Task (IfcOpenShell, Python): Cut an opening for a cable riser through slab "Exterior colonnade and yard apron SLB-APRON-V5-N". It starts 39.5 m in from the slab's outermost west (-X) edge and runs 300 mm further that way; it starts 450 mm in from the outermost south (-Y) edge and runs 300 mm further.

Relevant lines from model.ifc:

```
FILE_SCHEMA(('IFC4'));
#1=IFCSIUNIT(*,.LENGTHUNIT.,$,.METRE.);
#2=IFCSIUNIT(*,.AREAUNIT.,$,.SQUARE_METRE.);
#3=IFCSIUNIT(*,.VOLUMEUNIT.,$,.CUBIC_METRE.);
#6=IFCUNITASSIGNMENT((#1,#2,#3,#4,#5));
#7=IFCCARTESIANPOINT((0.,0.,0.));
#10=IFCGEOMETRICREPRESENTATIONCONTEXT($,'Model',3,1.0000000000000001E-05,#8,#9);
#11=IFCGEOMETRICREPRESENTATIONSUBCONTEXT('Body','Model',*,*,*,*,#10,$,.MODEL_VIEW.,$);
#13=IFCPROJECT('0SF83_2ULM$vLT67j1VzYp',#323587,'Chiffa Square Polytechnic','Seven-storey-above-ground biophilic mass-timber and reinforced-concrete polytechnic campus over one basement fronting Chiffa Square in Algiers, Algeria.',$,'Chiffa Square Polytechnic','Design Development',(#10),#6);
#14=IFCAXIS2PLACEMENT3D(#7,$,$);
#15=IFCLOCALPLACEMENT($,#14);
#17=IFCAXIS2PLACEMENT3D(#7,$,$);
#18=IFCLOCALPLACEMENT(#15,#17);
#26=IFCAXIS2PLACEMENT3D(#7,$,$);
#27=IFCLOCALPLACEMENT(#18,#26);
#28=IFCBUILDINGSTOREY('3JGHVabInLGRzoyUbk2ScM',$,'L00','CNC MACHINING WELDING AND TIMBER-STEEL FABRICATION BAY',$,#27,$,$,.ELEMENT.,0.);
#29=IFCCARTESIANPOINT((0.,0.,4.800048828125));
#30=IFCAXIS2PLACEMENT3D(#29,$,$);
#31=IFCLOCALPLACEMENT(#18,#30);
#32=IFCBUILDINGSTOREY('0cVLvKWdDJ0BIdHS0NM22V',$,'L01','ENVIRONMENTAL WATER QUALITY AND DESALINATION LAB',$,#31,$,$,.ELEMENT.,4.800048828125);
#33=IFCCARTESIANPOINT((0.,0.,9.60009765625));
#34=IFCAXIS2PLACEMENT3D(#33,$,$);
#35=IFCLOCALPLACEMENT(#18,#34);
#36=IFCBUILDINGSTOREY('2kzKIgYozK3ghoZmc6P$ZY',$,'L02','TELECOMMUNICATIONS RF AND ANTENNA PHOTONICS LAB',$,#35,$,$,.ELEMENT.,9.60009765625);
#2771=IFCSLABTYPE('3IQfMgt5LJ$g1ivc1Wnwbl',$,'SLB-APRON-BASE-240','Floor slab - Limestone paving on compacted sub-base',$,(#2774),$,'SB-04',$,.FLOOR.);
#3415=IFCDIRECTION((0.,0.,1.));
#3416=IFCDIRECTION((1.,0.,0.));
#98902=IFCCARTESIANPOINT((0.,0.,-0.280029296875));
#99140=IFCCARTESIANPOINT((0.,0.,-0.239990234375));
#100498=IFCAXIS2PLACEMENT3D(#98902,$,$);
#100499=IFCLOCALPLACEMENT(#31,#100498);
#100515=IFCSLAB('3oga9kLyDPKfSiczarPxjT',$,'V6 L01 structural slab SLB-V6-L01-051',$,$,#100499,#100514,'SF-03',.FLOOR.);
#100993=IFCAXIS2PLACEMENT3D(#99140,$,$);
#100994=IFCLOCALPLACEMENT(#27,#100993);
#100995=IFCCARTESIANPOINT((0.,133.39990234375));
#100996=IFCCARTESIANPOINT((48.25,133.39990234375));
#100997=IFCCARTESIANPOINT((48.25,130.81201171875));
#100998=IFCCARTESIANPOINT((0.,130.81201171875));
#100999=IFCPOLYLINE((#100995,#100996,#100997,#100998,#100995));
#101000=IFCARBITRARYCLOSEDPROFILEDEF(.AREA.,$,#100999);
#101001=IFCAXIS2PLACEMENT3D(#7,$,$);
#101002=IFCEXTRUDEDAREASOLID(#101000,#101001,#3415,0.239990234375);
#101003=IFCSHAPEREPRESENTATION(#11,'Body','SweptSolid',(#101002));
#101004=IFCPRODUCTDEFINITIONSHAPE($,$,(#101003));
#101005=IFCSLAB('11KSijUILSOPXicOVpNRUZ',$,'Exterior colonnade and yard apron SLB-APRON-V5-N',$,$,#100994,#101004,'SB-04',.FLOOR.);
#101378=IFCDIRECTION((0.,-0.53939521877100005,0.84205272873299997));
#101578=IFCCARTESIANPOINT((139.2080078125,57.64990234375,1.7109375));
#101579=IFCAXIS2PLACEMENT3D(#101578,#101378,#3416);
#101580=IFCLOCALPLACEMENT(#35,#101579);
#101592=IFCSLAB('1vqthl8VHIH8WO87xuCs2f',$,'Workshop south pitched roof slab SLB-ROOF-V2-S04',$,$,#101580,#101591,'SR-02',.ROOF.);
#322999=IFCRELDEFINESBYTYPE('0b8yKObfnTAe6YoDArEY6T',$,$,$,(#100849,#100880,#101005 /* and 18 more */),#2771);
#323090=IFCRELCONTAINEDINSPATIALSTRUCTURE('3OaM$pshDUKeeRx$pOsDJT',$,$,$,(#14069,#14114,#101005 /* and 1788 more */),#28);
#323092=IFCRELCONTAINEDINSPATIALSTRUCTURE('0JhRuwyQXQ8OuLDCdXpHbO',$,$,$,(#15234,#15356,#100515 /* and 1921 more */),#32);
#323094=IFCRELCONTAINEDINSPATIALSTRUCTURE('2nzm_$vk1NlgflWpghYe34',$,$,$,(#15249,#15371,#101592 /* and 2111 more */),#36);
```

```python
import numpy as np
import ifcopenshell
import ifcopenshell.api.feature
import ifcopenshell.api.geometry
import ifcopenshell.api.root
import ifcopenshell.geom
import ifcopenshell.util.placement
import ifcopenshell.util.representation
import ifcopenshell.util.shape
import ifcopenshell.util.unit

model = ifcopenshell.open("model.ifc")
unit_scale = ifcopenshell.util.unit.calculate_unit_scale(model)
settings = ifcopenshell.geom.settings()


def volume(element):
    """Net volume in cubic metres, openings subtracted."""
    shape = ifcopenshell.geom.create_shape(settings, element)
    return ifcopenshell.util.shape.get_volume(shape.geometry)


slab = model.by_guid("11KSijUILSOPXicOVpNRUZ")
before = volume(slab)

# Extent in the slab's own axes, in metres. The edges named are its -X and -Y sides.
slab_shape = ifcopenshell.geom.create_shape(settings, slab)
vertices = ifcopenshell.util.shape.get_vertices(slab_shape.geometry)
x_min, y_min, bottom = vertices.min(axis=0)
top = vertices[:, 2].max()

opening = ifcopenshell.api.root.create_entity(model, ifc_class="IfcOpeningElement", name="Cable riser opening", predefined_type="OPENING")
context = ifcopenshell.util.representation.get_context(model, "Model", "Body", "MODEL_VIEW")
width, depth = 0.3, 0.3
outline = [(0.0, 0.0), (width, 0.0), (width, depth), (0.0, depth), (0.0, 0.0)]
# Overshoot both faces by 50 mm so the cut is clean.
shape = ifcopenshell.api.geometry.add_slab_representation(
    model, context=context, depth=top - bottom + 0.1, polyline=outline
)
ifcopenshell.api.geometry.assign_representation(model, product=opening, representation=shape)

matrix = ifcopenshell.util.placement.get_local_placement(slab.ObjectPlacement)
matrix[:, 3] = matrix @ np.append(np.array([x_min + 39.5, y_min + 0.45, bottom - 0.05]) / unit_scale, 1.0)
ifcopenshell.api.geometry.edit_object_placement(model, product=opening, matrix=matrix, is_si=False)
ifcopenshell.api.feature.add_feature(model, feature=opening, element=slab)

after = volume(slab)

print(f"slab volume {before:.3f} -> {after:.3f} m3")

model.write("model-out.ifc")
```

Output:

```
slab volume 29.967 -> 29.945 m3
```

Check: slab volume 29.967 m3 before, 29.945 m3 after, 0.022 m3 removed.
